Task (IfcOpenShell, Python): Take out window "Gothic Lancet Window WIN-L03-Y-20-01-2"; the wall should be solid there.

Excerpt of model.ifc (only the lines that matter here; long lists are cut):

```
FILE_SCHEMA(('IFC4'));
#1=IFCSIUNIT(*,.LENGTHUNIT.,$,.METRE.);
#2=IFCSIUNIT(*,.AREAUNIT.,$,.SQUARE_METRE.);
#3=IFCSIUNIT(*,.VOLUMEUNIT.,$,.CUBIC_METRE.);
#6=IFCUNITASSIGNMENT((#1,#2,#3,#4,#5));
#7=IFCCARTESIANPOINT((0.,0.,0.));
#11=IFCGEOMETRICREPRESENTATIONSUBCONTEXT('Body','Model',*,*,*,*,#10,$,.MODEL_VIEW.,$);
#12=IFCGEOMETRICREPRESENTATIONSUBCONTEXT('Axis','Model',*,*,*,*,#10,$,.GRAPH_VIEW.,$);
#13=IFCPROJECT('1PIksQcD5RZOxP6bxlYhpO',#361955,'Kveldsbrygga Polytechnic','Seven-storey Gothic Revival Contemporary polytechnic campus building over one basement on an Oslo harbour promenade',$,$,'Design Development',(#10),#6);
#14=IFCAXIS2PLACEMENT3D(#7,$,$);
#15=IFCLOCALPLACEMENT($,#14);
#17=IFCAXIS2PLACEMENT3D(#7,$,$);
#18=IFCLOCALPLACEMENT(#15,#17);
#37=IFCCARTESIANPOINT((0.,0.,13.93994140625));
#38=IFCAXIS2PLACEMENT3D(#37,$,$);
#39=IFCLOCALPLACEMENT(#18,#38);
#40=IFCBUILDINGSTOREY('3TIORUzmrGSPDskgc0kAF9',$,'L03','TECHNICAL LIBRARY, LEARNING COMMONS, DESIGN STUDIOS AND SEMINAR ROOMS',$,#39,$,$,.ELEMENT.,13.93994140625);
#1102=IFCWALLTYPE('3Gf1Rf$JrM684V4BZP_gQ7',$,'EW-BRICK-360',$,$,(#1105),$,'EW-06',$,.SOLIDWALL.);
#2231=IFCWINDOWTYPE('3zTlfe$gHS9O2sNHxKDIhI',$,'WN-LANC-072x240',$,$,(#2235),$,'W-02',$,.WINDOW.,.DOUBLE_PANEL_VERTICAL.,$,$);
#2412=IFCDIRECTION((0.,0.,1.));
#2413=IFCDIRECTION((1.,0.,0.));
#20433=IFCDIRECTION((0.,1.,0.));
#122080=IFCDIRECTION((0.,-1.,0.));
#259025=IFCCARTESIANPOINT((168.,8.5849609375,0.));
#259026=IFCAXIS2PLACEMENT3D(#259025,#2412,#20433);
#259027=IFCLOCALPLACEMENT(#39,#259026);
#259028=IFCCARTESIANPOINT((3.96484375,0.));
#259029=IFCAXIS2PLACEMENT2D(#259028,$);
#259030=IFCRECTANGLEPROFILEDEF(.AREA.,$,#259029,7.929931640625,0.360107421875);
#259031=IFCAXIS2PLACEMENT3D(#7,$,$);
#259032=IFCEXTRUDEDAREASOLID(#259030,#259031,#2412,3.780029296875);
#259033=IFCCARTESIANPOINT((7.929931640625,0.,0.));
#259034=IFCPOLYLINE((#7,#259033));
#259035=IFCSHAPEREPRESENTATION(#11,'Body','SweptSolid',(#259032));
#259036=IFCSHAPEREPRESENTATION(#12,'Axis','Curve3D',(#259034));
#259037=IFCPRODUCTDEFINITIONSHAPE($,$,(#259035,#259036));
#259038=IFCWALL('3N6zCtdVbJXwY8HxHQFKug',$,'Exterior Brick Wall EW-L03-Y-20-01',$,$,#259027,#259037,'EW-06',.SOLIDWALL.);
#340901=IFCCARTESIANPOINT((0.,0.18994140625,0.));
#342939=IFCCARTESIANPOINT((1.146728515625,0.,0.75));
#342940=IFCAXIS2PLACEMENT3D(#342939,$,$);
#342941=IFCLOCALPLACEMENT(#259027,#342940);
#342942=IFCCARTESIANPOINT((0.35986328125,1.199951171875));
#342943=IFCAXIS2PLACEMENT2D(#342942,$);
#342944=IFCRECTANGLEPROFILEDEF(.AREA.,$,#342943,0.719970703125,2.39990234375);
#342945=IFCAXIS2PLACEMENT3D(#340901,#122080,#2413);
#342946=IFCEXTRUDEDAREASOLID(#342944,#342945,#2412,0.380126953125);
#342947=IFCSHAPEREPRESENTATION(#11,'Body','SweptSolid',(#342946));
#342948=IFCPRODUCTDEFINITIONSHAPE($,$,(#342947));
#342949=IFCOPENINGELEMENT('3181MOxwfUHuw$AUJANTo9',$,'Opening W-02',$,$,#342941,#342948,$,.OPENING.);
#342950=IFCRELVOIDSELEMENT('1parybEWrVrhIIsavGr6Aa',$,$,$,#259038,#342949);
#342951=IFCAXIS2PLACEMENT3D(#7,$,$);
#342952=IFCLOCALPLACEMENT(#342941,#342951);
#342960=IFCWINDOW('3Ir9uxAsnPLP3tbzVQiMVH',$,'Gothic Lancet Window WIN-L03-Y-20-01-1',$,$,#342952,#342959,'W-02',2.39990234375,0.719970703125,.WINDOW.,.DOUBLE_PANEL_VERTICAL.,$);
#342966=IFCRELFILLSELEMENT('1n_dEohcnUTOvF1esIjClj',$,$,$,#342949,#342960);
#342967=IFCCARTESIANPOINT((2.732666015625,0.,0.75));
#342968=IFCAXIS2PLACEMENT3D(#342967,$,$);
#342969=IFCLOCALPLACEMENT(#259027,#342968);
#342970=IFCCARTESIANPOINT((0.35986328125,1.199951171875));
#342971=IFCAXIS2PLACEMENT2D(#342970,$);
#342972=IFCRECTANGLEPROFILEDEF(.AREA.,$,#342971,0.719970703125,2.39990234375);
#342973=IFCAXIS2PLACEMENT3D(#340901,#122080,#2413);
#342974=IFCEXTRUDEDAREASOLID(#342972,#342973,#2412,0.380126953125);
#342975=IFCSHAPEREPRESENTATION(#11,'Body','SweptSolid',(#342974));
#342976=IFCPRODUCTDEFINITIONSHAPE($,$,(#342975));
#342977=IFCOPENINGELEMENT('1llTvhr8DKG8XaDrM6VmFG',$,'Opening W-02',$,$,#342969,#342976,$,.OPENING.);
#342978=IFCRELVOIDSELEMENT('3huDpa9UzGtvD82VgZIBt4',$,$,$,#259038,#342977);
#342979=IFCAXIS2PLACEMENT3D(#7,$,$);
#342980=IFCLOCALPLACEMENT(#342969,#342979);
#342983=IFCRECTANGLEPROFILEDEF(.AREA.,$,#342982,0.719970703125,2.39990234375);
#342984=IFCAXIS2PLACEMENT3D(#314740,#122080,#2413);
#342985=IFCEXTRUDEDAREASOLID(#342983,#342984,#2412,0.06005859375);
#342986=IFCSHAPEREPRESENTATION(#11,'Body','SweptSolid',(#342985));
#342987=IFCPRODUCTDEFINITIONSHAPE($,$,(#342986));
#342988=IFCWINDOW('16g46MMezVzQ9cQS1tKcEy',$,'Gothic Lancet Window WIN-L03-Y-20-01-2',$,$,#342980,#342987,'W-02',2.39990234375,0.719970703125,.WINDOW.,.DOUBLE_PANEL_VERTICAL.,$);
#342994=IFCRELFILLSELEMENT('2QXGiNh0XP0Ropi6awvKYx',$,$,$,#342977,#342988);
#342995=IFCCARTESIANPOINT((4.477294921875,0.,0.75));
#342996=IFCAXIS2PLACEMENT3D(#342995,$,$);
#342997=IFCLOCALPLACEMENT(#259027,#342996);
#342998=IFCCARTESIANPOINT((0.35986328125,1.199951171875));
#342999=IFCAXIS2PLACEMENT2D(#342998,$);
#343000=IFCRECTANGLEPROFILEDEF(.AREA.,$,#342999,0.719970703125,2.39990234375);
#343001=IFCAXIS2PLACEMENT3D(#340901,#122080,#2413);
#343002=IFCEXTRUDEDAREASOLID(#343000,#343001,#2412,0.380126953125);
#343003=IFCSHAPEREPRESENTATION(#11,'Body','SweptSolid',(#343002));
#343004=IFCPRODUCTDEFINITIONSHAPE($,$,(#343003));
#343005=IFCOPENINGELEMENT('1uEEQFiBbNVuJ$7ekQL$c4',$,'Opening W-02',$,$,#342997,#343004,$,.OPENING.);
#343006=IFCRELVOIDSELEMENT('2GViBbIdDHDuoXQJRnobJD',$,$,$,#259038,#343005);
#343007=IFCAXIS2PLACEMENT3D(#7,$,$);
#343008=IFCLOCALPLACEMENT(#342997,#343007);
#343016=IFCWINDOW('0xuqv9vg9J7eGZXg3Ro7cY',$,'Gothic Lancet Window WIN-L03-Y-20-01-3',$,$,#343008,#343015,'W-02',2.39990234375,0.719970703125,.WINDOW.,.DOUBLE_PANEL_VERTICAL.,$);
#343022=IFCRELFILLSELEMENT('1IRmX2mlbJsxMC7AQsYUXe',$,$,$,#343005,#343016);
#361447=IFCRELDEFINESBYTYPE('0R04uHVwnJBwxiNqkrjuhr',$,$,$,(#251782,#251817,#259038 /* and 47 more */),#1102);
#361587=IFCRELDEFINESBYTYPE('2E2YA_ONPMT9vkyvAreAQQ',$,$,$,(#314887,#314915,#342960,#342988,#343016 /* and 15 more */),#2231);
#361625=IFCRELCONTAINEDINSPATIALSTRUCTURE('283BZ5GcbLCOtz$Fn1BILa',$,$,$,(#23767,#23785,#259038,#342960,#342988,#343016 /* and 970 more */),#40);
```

```python
import ifcopenshell
import ifcopenshell.api.feature
import ifcopenshell.api.root
import ifcopenshell.geom
import ifcopenshell.util.shape

model = ifcopenshell.open("model.ifc")
settings = ifcopenshell.geom.settings()


def volume(element):
    """Net volume in cubic metres, openings subtracted."""
    shape = ifcopenshell.geom.create_shape(settings, element)
    return ifcopenshell.util.shape.get_volume(shape.geometry)


window = model.by_guid("16g46MMezVzQ9cQS1tKcEy")
opening = window.FillsVoids[0].RelatingOpeningElement
wall = opening.VoidsElements[0].RelatingBuildingElement
before = volume(wall)

ifcopenshell.api.root.remove_product(model, product=window)
ifcopenshell.api.feature.remove_feature(model, feature=opening)

after = volume(wall)

print(f"wall volume {before:.3f} -> {after:.3f} m3")

model.write("model_edited.ifc")
```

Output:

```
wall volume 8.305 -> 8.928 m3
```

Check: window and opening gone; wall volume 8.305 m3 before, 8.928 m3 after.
